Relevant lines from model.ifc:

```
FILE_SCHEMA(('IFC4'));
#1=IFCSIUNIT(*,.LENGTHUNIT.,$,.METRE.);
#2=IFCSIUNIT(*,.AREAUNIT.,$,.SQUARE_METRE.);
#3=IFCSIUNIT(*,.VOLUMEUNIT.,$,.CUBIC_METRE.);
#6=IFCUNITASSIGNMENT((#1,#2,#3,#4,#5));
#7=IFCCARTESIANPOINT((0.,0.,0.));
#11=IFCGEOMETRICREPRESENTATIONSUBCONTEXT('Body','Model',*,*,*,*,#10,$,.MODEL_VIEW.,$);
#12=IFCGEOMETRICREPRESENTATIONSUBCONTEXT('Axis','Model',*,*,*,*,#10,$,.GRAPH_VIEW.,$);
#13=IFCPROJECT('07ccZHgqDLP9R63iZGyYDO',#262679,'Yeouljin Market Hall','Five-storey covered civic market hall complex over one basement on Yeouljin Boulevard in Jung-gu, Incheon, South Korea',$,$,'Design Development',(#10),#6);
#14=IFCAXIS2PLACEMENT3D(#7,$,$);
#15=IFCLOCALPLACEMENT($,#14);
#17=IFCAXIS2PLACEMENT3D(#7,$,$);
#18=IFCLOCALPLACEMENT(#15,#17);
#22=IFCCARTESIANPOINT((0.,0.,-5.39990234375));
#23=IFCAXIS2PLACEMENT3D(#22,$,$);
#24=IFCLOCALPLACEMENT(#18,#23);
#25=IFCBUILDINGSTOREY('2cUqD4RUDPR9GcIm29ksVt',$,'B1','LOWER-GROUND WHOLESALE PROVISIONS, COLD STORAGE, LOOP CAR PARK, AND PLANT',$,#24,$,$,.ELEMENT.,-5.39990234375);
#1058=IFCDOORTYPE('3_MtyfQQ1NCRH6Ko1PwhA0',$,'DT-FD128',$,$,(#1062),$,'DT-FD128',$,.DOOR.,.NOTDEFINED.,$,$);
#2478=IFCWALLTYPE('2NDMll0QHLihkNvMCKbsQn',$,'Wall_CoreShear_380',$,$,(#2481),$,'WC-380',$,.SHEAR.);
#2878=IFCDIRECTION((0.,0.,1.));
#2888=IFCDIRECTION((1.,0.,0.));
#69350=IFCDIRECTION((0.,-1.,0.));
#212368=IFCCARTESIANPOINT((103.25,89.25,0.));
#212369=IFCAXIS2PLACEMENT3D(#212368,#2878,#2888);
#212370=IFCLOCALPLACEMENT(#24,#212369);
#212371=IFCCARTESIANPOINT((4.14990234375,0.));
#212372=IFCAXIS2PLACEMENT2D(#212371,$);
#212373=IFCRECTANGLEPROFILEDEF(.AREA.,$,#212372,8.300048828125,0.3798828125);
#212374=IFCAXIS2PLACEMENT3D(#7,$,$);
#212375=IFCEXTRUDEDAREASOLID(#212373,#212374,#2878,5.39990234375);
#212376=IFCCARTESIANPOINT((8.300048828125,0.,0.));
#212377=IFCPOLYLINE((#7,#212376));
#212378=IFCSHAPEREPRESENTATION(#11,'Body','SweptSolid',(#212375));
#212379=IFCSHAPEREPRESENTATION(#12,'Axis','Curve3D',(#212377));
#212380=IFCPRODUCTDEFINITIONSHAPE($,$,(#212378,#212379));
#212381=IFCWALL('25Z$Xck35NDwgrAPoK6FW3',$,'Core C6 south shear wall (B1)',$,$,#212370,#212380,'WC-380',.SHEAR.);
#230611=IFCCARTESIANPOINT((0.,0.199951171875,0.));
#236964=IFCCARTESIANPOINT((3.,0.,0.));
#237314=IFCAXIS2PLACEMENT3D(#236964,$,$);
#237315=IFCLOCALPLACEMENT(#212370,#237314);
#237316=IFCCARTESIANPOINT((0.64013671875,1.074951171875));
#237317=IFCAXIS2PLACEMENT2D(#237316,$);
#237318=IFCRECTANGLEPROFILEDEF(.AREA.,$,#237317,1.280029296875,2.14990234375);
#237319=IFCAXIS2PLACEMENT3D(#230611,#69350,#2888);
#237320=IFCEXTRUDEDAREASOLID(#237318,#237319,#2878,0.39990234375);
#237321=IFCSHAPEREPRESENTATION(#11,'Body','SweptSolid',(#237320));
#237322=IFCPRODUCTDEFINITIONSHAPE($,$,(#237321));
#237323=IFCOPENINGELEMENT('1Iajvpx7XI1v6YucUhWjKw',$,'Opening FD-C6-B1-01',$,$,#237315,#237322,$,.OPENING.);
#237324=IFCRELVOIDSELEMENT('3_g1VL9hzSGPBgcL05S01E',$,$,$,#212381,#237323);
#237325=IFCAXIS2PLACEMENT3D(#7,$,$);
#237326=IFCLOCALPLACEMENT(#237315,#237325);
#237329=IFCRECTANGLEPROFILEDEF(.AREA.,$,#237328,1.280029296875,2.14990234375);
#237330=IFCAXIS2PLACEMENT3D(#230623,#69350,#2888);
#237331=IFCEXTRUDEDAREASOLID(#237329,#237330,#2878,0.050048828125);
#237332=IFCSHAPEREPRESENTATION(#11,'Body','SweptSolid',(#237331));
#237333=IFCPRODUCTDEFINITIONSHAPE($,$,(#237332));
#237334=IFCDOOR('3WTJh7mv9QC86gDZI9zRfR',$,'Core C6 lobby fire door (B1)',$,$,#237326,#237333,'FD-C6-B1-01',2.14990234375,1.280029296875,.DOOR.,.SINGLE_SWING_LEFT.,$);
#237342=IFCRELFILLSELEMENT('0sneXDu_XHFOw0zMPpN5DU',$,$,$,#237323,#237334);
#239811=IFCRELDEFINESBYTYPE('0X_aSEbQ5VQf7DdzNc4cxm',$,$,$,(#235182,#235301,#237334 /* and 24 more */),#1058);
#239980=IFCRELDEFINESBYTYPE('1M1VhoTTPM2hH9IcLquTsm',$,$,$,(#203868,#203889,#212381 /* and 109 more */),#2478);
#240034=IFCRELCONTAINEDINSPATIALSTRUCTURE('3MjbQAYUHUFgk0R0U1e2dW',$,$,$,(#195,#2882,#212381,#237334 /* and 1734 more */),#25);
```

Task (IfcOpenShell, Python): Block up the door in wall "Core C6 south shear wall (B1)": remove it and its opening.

```python
import ifcopenshell
import ifcopenshell.api.feature
import ifcopenshell.api.root
import ifcopenshell.geom
import ifcopenshell.util.shape

model = ifcopenshell.open("model.ifc")
settings = ifcopenshell.geom.settings()


def volume(element):
    """Net volume in cubic metres, openings subtracted."""
    shape = ifcopenshell.geom.create_shape(settings, element)
    return ifcopenshell.util.shape.get_volume(shape.geometry)


door = model.by_guid("3WTJh7mv9QC86gDZI9zRfR")
opening = door.FillsVoids[0].RelatingOpeningElement
wall = opening.VoidsElements[0].RelatingBuildingElement
before = volume(wall)

ifcopenshell.api.root.remove_product(model, product=door)
ifcopenshell.api.feature.remove_feature(model, feature=opening)

after = volume(wall)

print(f"wall volume {before:.3f} -> {after:.3f} m3")

model.write("model_v2.ifc")
```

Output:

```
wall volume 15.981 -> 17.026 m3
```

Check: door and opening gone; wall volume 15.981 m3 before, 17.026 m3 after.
